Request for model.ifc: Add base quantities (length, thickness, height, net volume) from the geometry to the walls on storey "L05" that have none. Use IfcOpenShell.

First a look at what the model holds.

```python
import ifcopenshell
import ifcopenshell.util.element
import ifcopenshell.util.unit

model = ifcopenshell.open("model.ifc")
print(model.schema)
for unit_type in ("LENGTHUNIT", "AREAUNIT", "VOLUMEUNIT"):
    print(unit_type, ifcopenshell.util.unit.calculate_unit_scale(model, unit_type))
storey = next(s for s in model.by_type("IfcBuildingStorey") if s.Name == "L05")
walls = [e for e in ifcopenshell.util.element.get_decomposition(storey) if e.is_a("IfcWall")]
for e in sorted(walls, key=lambda e: e.id()):
    print(e.id(), e.is_a(), e.Name, list(ifcopenshell.util.element.get_psets(e, qtos_only=True)), sep=" | ")
```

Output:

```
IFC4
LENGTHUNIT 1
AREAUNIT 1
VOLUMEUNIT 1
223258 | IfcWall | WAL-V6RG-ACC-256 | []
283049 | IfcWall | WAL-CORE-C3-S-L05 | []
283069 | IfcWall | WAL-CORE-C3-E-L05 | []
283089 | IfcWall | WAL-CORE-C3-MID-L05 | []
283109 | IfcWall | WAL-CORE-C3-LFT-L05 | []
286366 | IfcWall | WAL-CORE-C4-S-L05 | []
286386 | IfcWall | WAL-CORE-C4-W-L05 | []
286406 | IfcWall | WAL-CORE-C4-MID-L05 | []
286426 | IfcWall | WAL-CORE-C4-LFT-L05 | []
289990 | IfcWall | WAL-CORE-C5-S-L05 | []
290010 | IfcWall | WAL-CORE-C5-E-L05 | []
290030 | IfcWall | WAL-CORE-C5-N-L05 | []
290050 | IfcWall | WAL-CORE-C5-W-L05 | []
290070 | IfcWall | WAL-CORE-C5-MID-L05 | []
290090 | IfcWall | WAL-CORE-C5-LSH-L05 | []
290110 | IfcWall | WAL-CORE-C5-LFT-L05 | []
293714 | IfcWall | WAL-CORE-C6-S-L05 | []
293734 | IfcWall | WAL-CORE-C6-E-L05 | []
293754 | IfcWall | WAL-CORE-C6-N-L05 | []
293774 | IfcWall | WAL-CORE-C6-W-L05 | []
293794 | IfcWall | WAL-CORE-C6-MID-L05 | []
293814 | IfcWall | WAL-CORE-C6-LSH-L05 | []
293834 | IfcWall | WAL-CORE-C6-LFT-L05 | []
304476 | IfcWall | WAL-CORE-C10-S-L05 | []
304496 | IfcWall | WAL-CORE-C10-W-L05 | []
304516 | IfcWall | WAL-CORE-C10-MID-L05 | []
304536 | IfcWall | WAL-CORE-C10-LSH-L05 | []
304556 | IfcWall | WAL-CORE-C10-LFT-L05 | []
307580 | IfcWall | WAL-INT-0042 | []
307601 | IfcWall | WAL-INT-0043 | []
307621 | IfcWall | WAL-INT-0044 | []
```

```python
import ifcopenshell
import ifcopenshell.api.pset
import ifcopenshell.geom
import ifcopenshell.util.element
import ifcopenshell.util.shape
import ifcopenshell.util.unit

model = ifcopenshell.open("model.ifc")
unit_scale = ifcopenshell.util.unit.calculate_unit_scale(model)
volume_scale = ifcopenshell.util.unit.calculate_unit_scale(model, "VOLUMEUNIT")
settings = ifcopenshell.geom.settings()

storey = next(s for s in model.by_type("IfcBuildingStorey") if s.Name == "L05")
walls = [e for e in ifcopenshell.util.element.get_decomposition(storey) if e.is_a("IfcWall")]

for e in sorted(walls, key=lambda e: e.id()):
    if ifcopenshell.util.element.get_psets(e, qtos_only=True, should_inherit=False):
        continue
    # Geometry comes back in metres, in the element's own axes.
    shape = ifcopenshell.geom.create_shape(settings, e)
    values = {
        "Length": ifcopenshell.util.shape.get_x(shape.geometry) / unit_scale,
        "Width": ifcopenshell.util.shape.get_y(shape.geometry) / unit_scale,
        "Height": ifcopenshell.util.shape.get_z(shape.geometry) / unit_scale,
        "NetVolume": ifcopenshell.util.shape.get_volume(shape.geometry) / volume_scale,
    }
    qto = ifcopenshell.api.pset.add_qto(model, product=e, name="Qto_WallBaseQuantities")
    ifcopenshell.api.pset.edit_qto(model, qto=qto, properties=values)
    print(e.id(), {k: round(v, 3) for k, v in values.items()})

model.write("model-out.ifc")
```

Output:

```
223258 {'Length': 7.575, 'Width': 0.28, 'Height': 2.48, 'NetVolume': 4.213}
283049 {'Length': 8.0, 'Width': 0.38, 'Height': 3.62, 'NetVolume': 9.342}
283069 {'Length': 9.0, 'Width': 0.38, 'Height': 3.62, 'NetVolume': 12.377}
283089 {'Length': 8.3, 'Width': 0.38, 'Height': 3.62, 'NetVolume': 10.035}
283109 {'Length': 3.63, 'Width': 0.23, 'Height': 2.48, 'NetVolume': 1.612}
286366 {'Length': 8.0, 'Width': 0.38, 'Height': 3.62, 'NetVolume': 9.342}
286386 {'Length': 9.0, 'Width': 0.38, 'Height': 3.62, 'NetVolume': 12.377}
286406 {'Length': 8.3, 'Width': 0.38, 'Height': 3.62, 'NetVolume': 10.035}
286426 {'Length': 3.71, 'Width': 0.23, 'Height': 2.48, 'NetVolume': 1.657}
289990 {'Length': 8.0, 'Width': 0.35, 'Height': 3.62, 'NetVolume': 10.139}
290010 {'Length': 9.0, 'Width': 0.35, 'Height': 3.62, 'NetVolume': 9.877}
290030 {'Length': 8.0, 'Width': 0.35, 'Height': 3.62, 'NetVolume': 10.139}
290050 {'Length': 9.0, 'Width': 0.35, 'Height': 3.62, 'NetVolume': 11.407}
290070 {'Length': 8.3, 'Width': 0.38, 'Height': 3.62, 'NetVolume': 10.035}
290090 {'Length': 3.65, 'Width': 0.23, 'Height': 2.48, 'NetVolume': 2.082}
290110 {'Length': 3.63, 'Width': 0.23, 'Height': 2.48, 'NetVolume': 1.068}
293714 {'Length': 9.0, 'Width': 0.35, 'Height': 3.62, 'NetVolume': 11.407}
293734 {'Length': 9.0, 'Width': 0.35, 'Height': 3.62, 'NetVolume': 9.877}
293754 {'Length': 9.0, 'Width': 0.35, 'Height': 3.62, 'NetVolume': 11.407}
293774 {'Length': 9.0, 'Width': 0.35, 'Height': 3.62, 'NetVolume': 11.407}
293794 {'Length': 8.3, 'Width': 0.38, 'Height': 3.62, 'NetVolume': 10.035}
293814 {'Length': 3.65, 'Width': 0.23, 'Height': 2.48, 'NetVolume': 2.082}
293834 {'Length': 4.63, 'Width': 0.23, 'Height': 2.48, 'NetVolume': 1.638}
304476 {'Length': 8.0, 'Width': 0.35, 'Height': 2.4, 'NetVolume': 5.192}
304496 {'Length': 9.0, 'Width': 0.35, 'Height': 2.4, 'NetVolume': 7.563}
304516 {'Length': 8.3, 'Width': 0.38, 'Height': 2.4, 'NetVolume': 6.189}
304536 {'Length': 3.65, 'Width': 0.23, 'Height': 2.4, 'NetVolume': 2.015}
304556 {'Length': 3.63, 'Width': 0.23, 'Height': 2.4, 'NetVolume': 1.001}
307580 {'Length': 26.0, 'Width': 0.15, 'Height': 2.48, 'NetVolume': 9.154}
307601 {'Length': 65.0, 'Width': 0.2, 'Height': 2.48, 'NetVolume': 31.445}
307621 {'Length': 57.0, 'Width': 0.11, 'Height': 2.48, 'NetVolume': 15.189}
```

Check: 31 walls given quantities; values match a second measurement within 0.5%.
